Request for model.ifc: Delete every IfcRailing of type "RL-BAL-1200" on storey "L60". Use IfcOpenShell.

First a look at what the model holds.

```python
import ifcopenshell
import ifcopenshell.util.element

model = ifcopenshell.open("model.ifc")
print(model.schema)
storey = next(s for s in model.by_type("IfcBuildingStorey") if s.Name == "L60")
railings = [e for e in ifcopenshell.util.element.get_decomposition(storey) if e.is_a("IfcRailing")]
seen = {}
for e in railings:
    element_type = ifcopenshell.util.element.get_type(e)
    name = element_type.Name if element_type not in (None, e) else None
    seen[name] = seen.get(name, 0) + 1
for name, count in sorted(seen.items(), key=str):
    print(count, "x", name)
```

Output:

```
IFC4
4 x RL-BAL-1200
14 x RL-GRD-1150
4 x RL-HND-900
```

```python
import ifcopenshell
import ifcopenshell.api.root
import ifcopenshell.util.element

model = ifcopenshell.open("model.ifc")

storey = next(s for s in model.by_type("IfcBuildingStorey") if s.Name == "L60")
railings = [e for e in ifcopenshell.util.element.get_decomposition(storey) if e.is_a("IfcRailing")]
targets = [e for e in railings if (t := ifcopenshell.util.element.get_type(e)) not in (None, e) and t.Name == "RL-BAL-1200"]

for e in targets:
    ifcopenshell.api.root.remove_product(model, product=e)
print(len(targets), "removed")

model.write("model_v2.ifc")
```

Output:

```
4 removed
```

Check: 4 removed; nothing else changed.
